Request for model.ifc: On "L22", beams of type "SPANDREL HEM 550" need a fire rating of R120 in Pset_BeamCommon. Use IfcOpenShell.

First a look at what the model holds.

```python
import ifcopenshell
import ifcopenshell.util.element

model = ifcopenshell.open("model.ifc")
print(model.schema)
storey = next(s for s in model.by_type("IfcBuildingStorey") if s.Name == "L22")
beams = [e for e in ifcopenshell.util.element.get_decomposition(storey) if e.is_a("IfcBeam")]
seen = {}
for e in beams:
    element_type = ifcopenshell.util.element.get_type(e)
    key = (element_type.Name if element_type != e and element_type else None, ifcopenshell.util.element.get_pset(e, "Pset_BeamCommon", "FireRating"))
    seen[key] = seen.get(key, 0) + 1
for (name, value), count in sorted(seen.items(), key=str):
    print(count, "x", name, "|", value)
```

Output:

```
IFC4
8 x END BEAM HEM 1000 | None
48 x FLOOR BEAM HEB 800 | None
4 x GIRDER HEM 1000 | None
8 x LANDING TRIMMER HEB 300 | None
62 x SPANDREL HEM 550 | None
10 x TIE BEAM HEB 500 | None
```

```python
import ifcopenshell
import ifcopenshell.api.pset
import ifcopenshell.util.element

model = ifcopenshell.open("model.ifc")

storey = next(s for s in model.by_type("IfcBuildingStorey") if s.Name == "L22")
beams = [e for e in ifcopenshell.util.element.get_decomposition(storey) if e.is_a("IfcBeam")]

count = 0
for e in beams:
    element_type = ifcopenshell.util.element.get_type(e)
    if element_type in (None, e) or element_type.Name != "SPANDREL HEM 550":
        continue
    found = ifcopenshell.util.element.get_pset(e, "Pset_BeamCommon", should_inherit=False)
    if found:
        pset = model.by_id(found["id"])
        if len(ifcopenshell.util.element.get_elements_by_pset(pset)) > 1:
            pset = ifcopenshell.api.pset.unshare_pset(model, products=[e], pset=pset)[0]
    else:
        pset = ifcopenshell.api.pset.add_pset(model, product=e, name="Pset_BeamCommon")
    ifcopenshell.api.pset.edit_pset(model, pset=pset, properties={"FireRating": "R120"})
    count += 1

print(count, "beams updated")

model.write("model_rev.ifc")
```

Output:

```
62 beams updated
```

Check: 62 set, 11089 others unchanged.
